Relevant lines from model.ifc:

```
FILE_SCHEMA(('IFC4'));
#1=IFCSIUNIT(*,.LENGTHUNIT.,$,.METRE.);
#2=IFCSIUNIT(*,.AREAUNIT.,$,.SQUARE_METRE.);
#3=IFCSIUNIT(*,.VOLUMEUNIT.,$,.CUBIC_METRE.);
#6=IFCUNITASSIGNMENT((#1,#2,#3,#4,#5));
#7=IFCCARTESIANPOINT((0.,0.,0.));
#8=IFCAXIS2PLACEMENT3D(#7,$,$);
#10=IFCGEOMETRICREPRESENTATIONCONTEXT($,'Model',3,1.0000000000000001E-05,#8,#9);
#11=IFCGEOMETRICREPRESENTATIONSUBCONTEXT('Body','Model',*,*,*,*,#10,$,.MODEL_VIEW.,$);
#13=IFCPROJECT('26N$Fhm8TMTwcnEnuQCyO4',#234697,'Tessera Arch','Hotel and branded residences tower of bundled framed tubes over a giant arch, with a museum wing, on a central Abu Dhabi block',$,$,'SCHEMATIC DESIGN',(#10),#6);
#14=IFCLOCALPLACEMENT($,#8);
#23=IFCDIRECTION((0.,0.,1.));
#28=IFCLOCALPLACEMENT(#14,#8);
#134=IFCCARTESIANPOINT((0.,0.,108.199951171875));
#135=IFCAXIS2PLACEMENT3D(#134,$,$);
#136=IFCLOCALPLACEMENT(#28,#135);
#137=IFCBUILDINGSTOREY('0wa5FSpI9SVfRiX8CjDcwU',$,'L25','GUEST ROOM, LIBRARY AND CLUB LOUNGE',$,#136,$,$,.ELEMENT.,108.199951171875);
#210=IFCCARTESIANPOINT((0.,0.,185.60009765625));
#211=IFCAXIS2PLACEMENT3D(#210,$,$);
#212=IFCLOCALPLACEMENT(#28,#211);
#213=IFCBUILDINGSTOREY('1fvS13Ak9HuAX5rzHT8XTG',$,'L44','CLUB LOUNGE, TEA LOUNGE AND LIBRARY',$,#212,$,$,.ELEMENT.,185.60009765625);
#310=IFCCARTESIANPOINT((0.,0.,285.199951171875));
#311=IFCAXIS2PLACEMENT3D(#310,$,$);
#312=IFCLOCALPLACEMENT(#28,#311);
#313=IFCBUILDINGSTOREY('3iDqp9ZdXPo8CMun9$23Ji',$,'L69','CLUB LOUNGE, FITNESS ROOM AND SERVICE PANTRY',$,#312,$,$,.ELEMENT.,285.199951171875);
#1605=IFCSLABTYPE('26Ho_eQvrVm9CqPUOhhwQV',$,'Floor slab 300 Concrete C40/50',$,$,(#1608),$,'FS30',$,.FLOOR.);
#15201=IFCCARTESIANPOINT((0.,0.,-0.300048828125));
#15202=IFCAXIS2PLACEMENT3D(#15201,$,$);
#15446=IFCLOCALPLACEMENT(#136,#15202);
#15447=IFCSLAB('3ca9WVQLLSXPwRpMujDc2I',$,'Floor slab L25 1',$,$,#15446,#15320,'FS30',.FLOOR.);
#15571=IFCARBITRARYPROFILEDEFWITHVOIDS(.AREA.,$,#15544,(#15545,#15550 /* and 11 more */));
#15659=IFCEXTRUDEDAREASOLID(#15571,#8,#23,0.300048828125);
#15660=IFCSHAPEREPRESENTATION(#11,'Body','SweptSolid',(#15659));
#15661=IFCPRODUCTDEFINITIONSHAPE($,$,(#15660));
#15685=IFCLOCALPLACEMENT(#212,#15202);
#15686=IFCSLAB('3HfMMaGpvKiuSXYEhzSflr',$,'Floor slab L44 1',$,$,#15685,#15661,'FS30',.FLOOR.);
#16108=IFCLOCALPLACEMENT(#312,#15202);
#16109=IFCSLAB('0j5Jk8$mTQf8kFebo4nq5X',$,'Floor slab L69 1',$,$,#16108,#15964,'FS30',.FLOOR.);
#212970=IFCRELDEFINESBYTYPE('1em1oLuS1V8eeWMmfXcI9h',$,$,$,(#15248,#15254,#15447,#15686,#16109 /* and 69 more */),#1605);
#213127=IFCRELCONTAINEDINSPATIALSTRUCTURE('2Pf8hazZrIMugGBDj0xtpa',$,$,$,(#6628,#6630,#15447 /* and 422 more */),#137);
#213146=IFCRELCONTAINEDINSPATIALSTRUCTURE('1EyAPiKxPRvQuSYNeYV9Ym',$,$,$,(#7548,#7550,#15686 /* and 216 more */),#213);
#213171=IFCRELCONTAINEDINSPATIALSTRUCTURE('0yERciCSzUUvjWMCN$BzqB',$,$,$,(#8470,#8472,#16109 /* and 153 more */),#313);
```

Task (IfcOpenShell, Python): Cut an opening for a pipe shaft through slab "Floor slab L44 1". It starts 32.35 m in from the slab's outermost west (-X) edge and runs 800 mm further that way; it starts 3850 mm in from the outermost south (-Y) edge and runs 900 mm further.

```python
import numpy as np
import ifcopenshell
import ifcopenshell.api.feature
import ifcopenshell.api.geometry
import ifcopenshell.api.root
import ifcopenshell.geom
import ifcopenshell.util.placement
import ifcopenshell.util.representation
import ifcopenshell.util.shape
import ifcopenshell.util.unit

model = ifcopenshell.open("model.ifc")
unit_scale = ifcopenshell.util.unit.calculate_unit_scale(model)
settings = ifcopenshell.geom.settings()


def volume(element):
    """Net volume in cubic metres, openings subtracted."""
    shape = ifcopenshell.geom.create_shape(settings, element)
    return ifcopenshell.util.shape.get_volume(shape.geometry)


slab = model.by_id(15686)
before = volume(slab)

# Extent in the slab's own axes, in metres. The edges named are its -X and -Y sides.
slab_shape = ifcopenshell.geom.create_shape(settings, slab)
vertices = ifcopenshell.util.shape.get_vertices(slab_shape.geometry)
x_min, y_min, bottom = vertices.min(axis=0)
top = vertices[:, 2].max()

opening = ifcopenshell.api.root.create_entity(model, ifc_class="IfcOpeningElement", name="Pipe shaft opening", predefined_type="OPENING")
context = ifcopenshell.util.representation.get_context(model, "Model", "Body", "MODEL_VIEW")
width, depth = 0.8, 0.9
outline = [(0.0, 0.0), (width, 0.0), (width, depth), (0.0, depth), (0.0, 0.0)]
# Overshoot both faces by 50 mm so the cut is clean.
shape = ifcopenshell.api.geometry.add_slab_representation(
    model, context=context, depth=top - bottom + 0.1, polyline=outline
)
ifcopenshell.api.geometry.assign_representation(model, product=opening, representation=shape)

matrix = ifcopenshell.util.placement.get_local_placement(slab.ObjectPlacement)
matrix[:, 3] = matrix @ np.append(np.array([x_min + 32.35, y_min + 3.85, bottom - 0.05]) / unit_scale, 1.0)
ifcopenshell.api.geometry.edit_object_placement(model, product=opening, matrix=matrix, is_si=False)
ifcopenshell.api.feature.add_feature(model, feature=opening, element=slab)

after = volume(slab)

print(f"slab volume {before:.3f} -> {after:.3f} m3")

model.write("model_edited.ifc")
```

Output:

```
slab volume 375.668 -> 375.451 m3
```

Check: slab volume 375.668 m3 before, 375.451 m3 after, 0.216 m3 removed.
